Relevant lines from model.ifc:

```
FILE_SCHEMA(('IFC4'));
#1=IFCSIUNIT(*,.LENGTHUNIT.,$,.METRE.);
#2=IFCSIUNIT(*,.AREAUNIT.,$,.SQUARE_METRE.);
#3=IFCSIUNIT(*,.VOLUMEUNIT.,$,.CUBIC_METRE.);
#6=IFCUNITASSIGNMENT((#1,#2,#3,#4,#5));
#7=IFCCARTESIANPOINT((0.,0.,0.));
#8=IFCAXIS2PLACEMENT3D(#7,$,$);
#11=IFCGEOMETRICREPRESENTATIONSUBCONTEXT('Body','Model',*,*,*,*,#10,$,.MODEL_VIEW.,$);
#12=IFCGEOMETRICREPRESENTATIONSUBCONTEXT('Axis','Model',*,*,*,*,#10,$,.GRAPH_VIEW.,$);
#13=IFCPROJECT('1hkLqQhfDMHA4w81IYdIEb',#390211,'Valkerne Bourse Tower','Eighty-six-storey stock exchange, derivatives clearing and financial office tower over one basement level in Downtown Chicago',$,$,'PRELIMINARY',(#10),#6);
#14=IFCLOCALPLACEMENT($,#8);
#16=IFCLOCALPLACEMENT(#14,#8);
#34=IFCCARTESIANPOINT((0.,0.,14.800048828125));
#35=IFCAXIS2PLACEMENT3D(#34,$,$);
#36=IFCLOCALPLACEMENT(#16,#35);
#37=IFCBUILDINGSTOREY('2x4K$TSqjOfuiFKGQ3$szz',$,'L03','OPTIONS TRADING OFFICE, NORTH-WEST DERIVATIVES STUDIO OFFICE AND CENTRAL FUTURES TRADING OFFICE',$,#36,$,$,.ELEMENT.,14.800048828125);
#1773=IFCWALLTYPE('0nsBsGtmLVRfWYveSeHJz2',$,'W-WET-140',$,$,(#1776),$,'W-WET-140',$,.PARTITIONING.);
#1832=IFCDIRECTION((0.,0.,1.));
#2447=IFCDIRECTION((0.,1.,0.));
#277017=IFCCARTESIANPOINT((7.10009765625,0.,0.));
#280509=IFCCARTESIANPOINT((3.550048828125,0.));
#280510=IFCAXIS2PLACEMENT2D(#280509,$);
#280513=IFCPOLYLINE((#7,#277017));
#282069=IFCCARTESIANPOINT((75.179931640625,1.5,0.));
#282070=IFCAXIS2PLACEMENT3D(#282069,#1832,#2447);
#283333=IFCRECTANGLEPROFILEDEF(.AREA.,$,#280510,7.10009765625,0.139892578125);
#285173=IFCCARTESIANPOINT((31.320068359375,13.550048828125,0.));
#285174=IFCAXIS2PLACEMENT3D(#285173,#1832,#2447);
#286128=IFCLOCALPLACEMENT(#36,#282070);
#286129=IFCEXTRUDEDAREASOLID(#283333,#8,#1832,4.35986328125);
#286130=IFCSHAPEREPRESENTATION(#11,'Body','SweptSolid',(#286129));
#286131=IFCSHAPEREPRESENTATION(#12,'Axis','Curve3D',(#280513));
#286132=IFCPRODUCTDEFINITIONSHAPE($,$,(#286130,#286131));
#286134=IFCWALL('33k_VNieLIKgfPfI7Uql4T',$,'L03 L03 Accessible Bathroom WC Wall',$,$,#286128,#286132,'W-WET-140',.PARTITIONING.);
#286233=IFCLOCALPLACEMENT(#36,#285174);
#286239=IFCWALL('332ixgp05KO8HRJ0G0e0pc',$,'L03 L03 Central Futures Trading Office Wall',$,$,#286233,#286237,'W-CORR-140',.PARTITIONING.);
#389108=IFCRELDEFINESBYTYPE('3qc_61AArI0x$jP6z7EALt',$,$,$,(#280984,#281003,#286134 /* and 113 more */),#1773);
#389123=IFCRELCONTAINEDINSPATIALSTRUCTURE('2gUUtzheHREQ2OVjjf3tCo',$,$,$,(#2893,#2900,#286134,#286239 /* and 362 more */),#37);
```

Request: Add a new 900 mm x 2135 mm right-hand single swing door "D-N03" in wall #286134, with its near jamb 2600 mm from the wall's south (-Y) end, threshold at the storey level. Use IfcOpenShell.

```python
import numpy as np
import ifcopenshell
import ifcopenshell.api.feature
import ifcopenshell.api.geometry
import ifcopenshell.api.root
import ifcopenshell.api.spatial
import ifcopenshell.geom
import ifcopenshell.util.element
import ifcopenshell.util.placement
import ifcopenshell.util.representation
import ifcopenshell.util.shape
import ifcopenshell.util.unit

model = ifcopenshell.open("model.ifc")
unit_scale = ifcopenshell.util.unit.calculate_unit_scale(model)
settings = ifcopenshell.geom.settings()


def volume(element):
    """Net volume in cubic metres, openings subtracted."""
    shape = ifcopenshell.geom.create_shape(settings, element)
    return ifcopenshell.util.shape.get_volume(shape.geometry)


wall = model.by_guid("33k_VNieLIKgfPfI7Uql4T")
storey = ifcopenshell.util.element.get_container(wall, ifc_class="IfcBuildingStorey")
context = ifcopenshell.util.representation.get_context(model, "Model", "Body", "MODEL_VIEW")
before = volume(wall)

width, height, from_end, sill = 0.9, 2.135, 2.6, 0.0  # metres

# The wall runs along its own X axis, and the end named is its -X end.
wall_shape = ifcopenshell.geom.create_shape(settings, wall)
x, y, z = ifcopenshell.util.shape.get_vertices(wall_shape.geometry).T
start = x.min() + from_end
face, thickness = float(y.min()), float(y.max() - y.min())
wall_matrix = ifcopenshell.util.placement.get_local_placement(wall.ObjectPlacement)
level = ifcopenshell.util.placement.get_local_placement(storey.ObjectPlacement)[2, 3]


def in_wall(x, y):
    """Placement at x, y metres in the wall's axes, at sill height."""
    matrix = wall_matrix.copy()
    matrix[:, 3] = wall_matrix @ np.array([x / unit_scale, y / unit_scale, 0.0, 1.0])
    matrix[2, 3] = level + sill / unit_scale
    return matrix


# Opening: a box that overshoots both wall faces by 50 mm.
opening = ifcopenshell.api.root.create_entity(model, ifc_class="IfcOpeningElement", predefined_type="OPENING")
box = ifcopenshell.api.geometry.add_wall_representation(
    model, context=context, length=width, height=height, thickness=thickness + 0.1
)
ifcopenshell.api.geometry.assign_representation(model, product=opening, representation=box)
ifcopenshell.api.geometry.edit_object_placement(model, product=opening, matrix=in_wall(start, face - 0.05), is_si=False)
ifcopenshell.api.feature.add_feature(model, feature=opening, element=wall)

door = ifcopenshell.api.root.create_entity(model, ifc_class="IfcDoor", name="D-N03", predefined_type="DOOR")
door.OverallWidth, door.OverallHeight = width / unit_scale, height / unit_scale
door.OperationType = "SINGLE_SWING_RIGHT"
body = ifcopenshell.api.geometry.add_door_representation(
    model,
    context=context,
    overall_width=door.OverallWidth,
    overall_height=door.OverallHeight,
    operation_type="SINGLE_SWING_RIGHT",
    lining_properties={"LiningDepth": thickness / unit_scale, "ThresholdDepth": thickness / unit_scale},
)
ifcopenshell.api.geometry.assign_representation(model, product=door, representation=body)
ifcopenshell.api.spatial.assign_container(model, products=[door], relating_structure=storey)
ifcopenshell.api.feature.add_filling(model, opening=opening, element=door)

# The lining spans the wall, so the door starts at the wall face.
ifcopenshell.api.geometry.edit_object_placement(model, product=door, matrix=in_wall(start, face), is_si=False)

after = volume(wall)

print(f"wall volume {before:.3f} -> {after:.3f} m3")

model.write("model_edited.ifc")
```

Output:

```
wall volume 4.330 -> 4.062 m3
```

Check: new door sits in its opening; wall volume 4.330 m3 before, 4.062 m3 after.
